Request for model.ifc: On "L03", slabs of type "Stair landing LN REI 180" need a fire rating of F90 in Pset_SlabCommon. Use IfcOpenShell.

First a look at what the model holds.

```python
import ifcopenshell
import ifcopenshell.util.element

model = ifcopenshell.open("model.ifc")
print(model.schema)
storey = next(s for s in model.by_type("IfcBuildingStorey") if s.Name == "L03")
slabs = [e for e in ifcopenshell.util.element.get_decomposition(storey) if e.is_a("IfcSlab")]
seen = {}
for e in slabs:
    element_type = ifcopenshell.util.element.get_type(e)
    key = (element_type.Name if element_type != e and element_type else None, ifcopenshell.util.element.get_pset(e, "Pset_SlabCommon", "FireRating"))
    seen[key] = seen.get(key, 0) + 1
for (name, value), count in sorted(seen.items(), key=str):
    print(count, "x", name, "|", value)
```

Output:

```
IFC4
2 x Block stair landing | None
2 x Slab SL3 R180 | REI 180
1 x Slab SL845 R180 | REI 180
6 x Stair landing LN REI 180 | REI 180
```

```python
import ifcopenshell
import ifcopenshell.api.pset
import ifcopenshell.util.element

model = ifcopenshell.open("model.ifc")

storey = next(s for s in model.by_type("IfcBuildingStorey") if s.Name == "L03")
slabs = [e for e in ifcopenshell.util.element.get_decomposition(storey) if e.is_a("IfcSlab")]

count = 0
for e in slabs:
    element_type = ifcopenshell.util.element.get_type(e)
    if element_type in (None, e) or element_type.Name != "Stair landing LN REI 180":
        continue
    # add_pset returns the element's existing set when there is one.
    pset = ifcopenshell.api.pset.add_pset(model, product=e, name="Pset_SlabCommon")
    ifcopenshell.api.pset.edit_pset(model, pset=pset, properties={"FireRating": "F90"})
    count += 1

print(count, "slabs updated")

model.write("model_v2.ifc")
```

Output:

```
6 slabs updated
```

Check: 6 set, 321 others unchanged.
